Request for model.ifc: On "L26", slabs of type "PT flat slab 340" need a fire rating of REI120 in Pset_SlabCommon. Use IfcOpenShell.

First a look at what the model holds.

```python
import ifcopenshell
import ifcopenshell.util.element

model = ifcopenshell.open("model.ifc")
print(model.schema)
storey = next(s for s in model.by_type("IfcBuildingStorey") if s.Name == "L26")
slabs = [e for e in ifcopenshell.util.element.get_decomposition(storey) if e.is_a("IfcSlab")]
seen = {}
for e in slabs:
    element_type = ifcopenshell.util.element.get_type(e)
    key = (element_type.Name if element_type != e and element_type else None, ifcopenshell.util.element.get_pset(e, "Pset_SlabCommon", "FireRating"))
    seen[key] = seen.get(key, 0) + 1
for (name, value), count in sorted(seen.items(), key=str):
    print(count, "x", name, "|", value)
```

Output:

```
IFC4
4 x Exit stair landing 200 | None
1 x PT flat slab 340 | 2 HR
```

```python
import ifcopenshell
import ifcopenshell.api.pset
import ifcopenshell.util.element

model = ifcopenshell.open("model.ifc")

storey = next(s for s in model.by_type("IfcBuildingStorey") if s.Name == "L26")
slabs = [e for e in ifcopenshell.util.element.get_decomposition(storey) if e.is_a("IfcSlab")]

count = 0
for e in slabs:
    element_type = ifcopenshell.util.element.get_type(e)
    if element_type in (None, e) or element_type.Name != "PT flat slab 340":
        continue
    found = ifcopenshell.util.element.get_pset(e, "Pset_SlabCommon", should_inherit=False)
    if found:
        pset = model.by_id(found["id"])
        if len(ifcopenshell.util.element.get_elements_by_pset(pset)) > 1:
            pset = ifcopenshell.api.pset.unshare_pset(model, products=[e], pset=pset)[0]
    else:
        pset = ifcopenshell.api.pset.add_pset(model, product=e, name="Pset_SlabCommon")
    ifcopenshell.api.pset.edit_pset(model, pset=pset, properties={"FireRating": "REI120"})
    count += 1

print(count, "slabs updated")

model.write("model_rev.ifc")
```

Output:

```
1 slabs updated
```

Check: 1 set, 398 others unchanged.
